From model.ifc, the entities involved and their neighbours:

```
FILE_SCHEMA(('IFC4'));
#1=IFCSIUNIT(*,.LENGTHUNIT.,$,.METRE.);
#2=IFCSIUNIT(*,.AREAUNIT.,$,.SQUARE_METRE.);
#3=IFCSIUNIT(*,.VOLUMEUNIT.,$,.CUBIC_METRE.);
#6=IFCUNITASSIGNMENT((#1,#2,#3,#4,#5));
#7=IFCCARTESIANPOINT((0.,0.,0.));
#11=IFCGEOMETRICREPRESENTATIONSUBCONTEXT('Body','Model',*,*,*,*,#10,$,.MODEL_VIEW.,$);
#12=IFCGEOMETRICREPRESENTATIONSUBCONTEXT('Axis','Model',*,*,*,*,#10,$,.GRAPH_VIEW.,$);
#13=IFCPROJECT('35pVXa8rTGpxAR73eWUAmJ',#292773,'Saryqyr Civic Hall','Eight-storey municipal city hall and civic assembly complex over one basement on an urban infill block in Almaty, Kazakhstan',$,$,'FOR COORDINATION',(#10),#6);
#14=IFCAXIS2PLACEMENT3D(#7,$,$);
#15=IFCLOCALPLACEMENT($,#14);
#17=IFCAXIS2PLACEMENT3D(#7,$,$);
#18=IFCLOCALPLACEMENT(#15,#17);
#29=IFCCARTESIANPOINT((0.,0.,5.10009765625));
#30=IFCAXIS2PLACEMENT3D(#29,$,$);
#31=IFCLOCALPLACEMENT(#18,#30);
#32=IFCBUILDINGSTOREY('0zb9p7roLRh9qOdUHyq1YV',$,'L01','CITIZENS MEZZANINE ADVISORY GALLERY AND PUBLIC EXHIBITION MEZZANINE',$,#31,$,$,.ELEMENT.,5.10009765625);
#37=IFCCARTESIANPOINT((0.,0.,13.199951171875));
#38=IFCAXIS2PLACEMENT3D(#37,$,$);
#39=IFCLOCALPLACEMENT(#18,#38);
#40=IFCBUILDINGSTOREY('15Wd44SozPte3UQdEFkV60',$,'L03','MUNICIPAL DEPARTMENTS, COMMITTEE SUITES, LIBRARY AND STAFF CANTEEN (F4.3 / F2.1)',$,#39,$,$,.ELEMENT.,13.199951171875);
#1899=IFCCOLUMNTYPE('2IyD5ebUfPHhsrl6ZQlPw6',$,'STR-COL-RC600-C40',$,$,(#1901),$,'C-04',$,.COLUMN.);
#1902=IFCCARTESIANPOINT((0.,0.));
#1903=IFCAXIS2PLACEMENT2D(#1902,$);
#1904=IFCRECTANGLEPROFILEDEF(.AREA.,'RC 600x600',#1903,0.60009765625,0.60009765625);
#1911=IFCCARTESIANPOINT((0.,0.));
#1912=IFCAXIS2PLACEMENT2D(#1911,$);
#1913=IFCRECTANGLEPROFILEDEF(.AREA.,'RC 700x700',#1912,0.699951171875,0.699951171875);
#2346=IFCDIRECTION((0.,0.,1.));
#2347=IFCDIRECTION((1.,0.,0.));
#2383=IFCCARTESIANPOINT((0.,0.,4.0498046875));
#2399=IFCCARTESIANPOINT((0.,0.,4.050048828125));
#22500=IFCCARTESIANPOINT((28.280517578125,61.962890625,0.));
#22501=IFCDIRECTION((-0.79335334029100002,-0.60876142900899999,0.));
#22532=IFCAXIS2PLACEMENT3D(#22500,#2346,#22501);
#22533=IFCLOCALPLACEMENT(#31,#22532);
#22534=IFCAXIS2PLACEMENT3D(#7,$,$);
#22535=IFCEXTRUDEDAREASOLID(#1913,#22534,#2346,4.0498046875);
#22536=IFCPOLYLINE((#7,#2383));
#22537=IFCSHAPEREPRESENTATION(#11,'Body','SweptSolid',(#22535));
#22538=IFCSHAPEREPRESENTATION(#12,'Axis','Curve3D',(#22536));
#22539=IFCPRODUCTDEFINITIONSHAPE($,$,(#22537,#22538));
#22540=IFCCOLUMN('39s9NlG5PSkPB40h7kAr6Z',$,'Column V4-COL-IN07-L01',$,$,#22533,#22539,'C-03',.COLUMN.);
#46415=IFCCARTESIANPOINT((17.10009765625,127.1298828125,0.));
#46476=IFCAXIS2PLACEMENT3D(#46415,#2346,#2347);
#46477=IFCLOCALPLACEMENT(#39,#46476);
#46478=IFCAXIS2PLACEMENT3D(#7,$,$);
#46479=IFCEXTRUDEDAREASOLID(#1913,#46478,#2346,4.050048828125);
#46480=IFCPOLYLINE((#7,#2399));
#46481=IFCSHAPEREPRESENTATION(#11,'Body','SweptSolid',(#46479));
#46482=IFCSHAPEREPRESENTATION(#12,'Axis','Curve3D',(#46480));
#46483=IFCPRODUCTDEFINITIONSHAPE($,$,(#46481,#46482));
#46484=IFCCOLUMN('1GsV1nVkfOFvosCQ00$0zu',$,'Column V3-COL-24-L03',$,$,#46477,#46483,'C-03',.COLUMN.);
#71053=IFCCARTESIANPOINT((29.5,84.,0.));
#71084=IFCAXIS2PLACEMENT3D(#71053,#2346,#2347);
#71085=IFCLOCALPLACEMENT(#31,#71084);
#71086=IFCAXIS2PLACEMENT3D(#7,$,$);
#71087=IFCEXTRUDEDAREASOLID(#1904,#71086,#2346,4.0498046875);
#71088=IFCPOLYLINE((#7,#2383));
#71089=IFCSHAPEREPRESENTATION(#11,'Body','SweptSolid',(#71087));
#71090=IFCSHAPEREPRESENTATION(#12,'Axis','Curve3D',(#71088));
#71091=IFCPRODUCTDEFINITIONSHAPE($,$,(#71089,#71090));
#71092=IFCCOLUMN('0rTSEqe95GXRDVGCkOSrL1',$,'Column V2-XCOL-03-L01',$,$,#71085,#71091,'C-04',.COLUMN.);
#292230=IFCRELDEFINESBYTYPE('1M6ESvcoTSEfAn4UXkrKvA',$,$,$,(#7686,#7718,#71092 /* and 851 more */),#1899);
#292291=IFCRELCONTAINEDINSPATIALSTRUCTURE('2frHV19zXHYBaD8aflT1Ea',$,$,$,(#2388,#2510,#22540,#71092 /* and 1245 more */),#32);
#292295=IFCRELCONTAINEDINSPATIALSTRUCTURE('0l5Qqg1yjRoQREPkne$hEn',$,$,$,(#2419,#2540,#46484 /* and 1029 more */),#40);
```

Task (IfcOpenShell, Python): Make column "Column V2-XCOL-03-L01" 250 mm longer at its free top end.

```python
import numpy as np
import ifcopenshell
import ifcopenshell.util.representation

model = ifcopenshell.open("model.ifc")

member = model.by_guid("0rTSEqe95GXRDVGCkOSrL1")
change = 0.25

# The extrusion runs towards the end named, so only its depth changes.
body = ifcopenshell.util.representation.get_representation(member, "Model", "Body")
solid = body.Items[0]
old_length = solid.Depth
solid.Depth += change

# Move the axis end point with it.
axis = next(r for r in member.Representation.Representations if r.RepresentationIdentifier == "Axis").Items[0]
start, end = (np.array(p.Coordinates) for p in axis.Points)
end = end + (end - start) / np.linalg.norm(end - start) * change
point = model.createIfcCartesianPoint(end.tolist())
axis.Points = [axis.Points[0], point]

print(f"length {old_length:g} -> {solid.Depth:g}")

model.write("model_rev.ifc")
```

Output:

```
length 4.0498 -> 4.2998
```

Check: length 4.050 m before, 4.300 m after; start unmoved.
